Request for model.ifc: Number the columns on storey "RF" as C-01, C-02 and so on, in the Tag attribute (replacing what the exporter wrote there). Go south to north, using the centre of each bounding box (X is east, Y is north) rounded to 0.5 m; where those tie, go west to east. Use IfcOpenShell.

First a look at what the model holds.

```python
import ifcopenshell
import ifcopenshell.util.element
import ifcopenshell.util.placement

model = ifcopenshell.open("model.ifc")
print(model.schema)
storey = next(s for s in model.by_type("IfcBuildingStorey") if s.Name == "RF")
columns = [e for e in ifcopenshell.util.element.get_decomposition(storey) if e.is_a("IfcColumn")]
for e in sorted(columns, key=lambda e: e.id()):
    origin = ifcopenshell.util.placement.get_local_placement(e.ObjectPlacement)[:3, 3]
    print(e.id(), e.Tag, e.Name, origin.round(2) + 0.0, sep=" | ")
```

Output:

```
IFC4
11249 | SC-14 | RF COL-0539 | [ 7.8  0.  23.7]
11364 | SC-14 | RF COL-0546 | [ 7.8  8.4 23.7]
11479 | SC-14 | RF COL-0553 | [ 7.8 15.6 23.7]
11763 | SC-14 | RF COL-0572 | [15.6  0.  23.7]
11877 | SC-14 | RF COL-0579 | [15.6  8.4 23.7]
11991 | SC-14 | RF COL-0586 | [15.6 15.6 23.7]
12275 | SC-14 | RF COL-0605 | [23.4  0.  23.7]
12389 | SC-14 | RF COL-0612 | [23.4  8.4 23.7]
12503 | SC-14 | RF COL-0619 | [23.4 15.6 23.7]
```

```python
import ifcopenshell
import ifcopenshell.geom
import ifcopenshell.util.element
import ifcopenshell.util.shape

model = ifcopenshell.open("model.ifc")
settings = ifcopenshell.geom.settings()
settings.set("use-world-coords", True)


def centre(element):
    shape = ifcopenshell.geom.create_shape(settings, element)
    return ifcopenshell.util.shape.get_bbox_centroid(shape.geometry)


storey = next(s for s in model.by_type("IfcBuildingStorey") if s.Name == "RF")
columns = [e for e in ifcopenshell.util.element.get_decomposition(storey) if e.is_a("IfcColumn")]

# Insertion points can sit at a corner or the storey origin, so sort by the geometry (in metres).
centres = {e: centre(e) for e in columns}
columns.sort(key=lambda e: (round(centres[e][1] / 0.5), centres[e][0]))

for i, e in enumerate(columns, start=1):
    number = f"C-{i:02d}"
    e.Tag = number
    print(e.id(), number)

model.write("model_rev.ifc")
```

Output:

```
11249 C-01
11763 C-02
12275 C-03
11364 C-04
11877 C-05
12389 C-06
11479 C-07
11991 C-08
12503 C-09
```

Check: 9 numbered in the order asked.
